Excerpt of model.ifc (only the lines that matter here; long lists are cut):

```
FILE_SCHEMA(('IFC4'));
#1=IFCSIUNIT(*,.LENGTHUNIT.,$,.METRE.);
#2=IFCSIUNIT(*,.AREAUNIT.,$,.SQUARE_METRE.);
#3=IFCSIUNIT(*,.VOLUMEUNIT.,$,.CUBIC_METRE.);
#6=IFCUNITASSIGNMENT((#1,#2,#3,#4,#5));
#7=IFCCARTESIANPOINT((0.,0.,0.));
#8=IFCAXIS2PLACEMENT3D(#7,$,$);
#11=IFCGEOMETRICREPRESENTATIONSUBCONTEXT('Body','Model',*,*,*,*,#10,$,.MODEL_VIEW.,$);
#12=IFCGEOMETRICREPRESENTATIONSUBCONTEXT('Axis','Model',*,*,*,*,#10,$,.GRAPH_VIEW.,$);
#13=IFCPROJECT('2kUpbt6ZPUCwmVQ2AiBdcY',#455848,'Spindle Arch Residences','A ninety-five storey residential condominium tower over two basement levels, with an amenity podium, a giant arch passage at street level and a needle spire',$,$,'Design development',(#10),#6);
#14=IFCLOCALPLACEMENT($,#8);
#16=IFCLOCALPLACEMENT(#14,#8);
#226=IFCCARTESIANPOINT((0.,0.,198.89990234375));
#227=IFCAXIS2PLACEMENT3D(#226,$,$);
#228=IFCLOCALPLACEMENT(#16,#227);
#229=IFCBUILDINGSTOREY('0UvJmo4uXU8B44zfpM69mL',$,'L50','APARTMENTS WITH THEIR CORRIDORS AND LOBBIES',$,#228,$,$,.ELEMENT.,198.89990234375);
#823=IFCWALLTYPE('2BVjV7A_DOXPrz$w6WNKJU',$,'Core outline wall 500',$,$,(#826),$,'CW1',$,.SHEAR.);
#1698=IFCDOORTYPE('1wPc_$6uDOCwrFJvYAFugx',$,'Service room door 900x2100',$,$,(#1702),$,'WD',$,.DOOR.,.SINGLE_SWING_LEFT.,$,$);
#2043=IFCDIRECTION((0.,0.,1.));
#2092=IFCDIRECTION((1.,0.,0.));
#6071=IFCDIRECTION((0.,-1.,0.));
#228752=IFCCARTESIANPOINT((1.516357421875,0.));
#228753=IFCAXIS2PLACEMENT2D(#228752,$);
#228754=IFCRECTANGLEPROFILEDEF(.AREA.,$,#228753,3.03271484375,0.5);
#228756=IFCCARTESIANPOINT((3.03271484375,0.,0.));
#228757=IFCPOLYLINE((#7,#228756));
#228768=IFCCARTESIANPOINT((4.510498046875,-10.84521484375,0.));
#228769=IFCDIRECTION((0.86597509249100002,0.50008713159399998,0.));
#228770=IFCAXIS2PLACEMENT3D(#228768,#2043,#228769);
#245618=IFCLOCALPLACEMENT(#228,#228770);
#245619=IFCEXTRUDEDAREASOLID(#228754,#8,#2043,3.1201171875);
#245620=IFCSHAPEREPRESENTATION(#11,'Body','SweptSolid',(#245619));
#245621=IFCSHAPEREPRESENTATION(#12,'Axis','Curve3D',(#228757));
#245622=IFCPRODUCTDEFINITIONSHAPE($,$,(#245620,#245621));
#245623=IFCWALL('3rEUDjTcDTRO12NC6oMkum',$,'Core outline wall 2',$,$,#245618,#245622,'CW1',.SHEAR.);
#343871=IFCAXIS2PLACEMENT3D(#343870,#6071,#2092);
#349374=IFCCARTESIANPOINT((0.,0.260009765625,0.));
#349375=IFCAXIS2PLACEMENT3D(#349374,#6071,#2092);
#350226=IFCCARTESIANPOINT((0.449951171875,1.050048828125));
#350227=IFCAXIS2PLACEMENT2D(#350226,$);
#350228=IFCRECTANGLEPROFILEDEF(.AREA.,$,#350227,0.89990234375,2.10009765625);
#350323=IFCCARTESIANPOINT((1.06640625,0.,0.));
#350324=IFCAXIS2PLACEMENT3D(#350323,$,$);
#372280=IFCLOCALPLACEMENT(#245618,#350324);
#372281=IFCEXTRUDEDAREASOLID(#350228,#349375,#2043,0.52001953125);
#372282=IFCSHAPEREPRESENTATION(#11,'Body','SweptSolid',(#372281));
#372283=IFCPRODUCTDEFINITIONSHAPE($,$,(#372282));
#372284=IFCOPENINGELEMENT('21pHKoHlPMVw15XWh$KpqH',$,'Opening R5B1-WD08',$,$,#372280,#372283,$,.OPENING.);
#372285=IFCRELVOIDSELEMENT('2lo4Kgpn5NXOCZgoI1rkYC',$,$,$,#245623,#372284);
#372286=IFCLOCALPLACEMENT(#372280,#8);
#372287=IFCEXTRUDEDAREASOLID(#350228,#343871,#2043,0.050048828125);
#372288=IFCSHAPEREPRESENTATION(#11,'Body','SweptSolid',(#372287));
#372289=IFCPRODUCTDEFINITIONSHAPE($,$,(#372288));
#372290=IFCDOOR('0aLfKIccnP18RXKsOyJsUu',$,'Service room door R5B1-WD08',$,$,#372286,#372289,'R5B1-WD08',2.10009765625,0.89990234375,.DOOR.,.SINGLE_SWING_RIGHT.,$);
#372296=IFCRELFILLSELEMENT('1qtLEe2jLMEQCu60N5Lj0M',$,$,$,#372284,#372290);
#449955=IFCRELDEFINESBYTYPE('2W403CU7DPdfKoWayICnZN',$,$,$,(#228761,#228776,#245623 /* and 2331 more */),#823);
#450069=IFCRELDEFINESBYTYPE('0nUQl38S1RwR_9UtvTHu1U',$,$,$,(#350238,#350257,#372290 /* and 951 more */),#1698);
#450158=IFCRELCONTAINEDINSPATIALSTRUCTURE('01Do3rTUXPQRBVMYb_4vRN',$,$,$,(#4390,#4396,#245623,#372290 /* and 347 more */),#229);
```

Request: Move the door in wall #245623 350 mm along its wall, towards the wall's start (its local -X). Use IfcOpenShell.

```python
import ifcopenshell
import ifcopenshell.api.geometry
import ifcopenshell.util.placement
import ifcopenshell.util.unit

model = ifcopenshell.open("model.ifc")
unit_scale = ifcopenshell.util.unit.calculate_unit_scale(model)

door = model.by_id(372290)
opening = door.FillsVoids[0].RelatingOpeningElement
wall = opening.VoidsElements[0].RelatingBuildingElement

wall_matrix = ifcopenshell.util.placement.get_local_placement(wall.ObjectPlacement)
shift = wall_matrix[:3, 0] * -0.35 / unit_scale
before = ifcopenshell.util.placement.get_local_placement(door.ObjectPlacement)[:3, 3].copy()

# The door is placed relative to its opening, so it follows when the opening moves.
matrix = ifcopenshell.util.placement.get_local_placement(opening.ObjectPlacement)
matrix[:3, 3] += shift
ifcopenshell.api.geometry.edit_object_placement(
    model, product=opening, matrix=matrix, is_si=False, should_transform_children=True
)

after = ifcopenshell.util.placement.get_local_placement(door.ObjectPlacement)[:3, 3]
print("door moved by", (after - before).round(3) + 0.0)

model.write("model_v2.ifc")
```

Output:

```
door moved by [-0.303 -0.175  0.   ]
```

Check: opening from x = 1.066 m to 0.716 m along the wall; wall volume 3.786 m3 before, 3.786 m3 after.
